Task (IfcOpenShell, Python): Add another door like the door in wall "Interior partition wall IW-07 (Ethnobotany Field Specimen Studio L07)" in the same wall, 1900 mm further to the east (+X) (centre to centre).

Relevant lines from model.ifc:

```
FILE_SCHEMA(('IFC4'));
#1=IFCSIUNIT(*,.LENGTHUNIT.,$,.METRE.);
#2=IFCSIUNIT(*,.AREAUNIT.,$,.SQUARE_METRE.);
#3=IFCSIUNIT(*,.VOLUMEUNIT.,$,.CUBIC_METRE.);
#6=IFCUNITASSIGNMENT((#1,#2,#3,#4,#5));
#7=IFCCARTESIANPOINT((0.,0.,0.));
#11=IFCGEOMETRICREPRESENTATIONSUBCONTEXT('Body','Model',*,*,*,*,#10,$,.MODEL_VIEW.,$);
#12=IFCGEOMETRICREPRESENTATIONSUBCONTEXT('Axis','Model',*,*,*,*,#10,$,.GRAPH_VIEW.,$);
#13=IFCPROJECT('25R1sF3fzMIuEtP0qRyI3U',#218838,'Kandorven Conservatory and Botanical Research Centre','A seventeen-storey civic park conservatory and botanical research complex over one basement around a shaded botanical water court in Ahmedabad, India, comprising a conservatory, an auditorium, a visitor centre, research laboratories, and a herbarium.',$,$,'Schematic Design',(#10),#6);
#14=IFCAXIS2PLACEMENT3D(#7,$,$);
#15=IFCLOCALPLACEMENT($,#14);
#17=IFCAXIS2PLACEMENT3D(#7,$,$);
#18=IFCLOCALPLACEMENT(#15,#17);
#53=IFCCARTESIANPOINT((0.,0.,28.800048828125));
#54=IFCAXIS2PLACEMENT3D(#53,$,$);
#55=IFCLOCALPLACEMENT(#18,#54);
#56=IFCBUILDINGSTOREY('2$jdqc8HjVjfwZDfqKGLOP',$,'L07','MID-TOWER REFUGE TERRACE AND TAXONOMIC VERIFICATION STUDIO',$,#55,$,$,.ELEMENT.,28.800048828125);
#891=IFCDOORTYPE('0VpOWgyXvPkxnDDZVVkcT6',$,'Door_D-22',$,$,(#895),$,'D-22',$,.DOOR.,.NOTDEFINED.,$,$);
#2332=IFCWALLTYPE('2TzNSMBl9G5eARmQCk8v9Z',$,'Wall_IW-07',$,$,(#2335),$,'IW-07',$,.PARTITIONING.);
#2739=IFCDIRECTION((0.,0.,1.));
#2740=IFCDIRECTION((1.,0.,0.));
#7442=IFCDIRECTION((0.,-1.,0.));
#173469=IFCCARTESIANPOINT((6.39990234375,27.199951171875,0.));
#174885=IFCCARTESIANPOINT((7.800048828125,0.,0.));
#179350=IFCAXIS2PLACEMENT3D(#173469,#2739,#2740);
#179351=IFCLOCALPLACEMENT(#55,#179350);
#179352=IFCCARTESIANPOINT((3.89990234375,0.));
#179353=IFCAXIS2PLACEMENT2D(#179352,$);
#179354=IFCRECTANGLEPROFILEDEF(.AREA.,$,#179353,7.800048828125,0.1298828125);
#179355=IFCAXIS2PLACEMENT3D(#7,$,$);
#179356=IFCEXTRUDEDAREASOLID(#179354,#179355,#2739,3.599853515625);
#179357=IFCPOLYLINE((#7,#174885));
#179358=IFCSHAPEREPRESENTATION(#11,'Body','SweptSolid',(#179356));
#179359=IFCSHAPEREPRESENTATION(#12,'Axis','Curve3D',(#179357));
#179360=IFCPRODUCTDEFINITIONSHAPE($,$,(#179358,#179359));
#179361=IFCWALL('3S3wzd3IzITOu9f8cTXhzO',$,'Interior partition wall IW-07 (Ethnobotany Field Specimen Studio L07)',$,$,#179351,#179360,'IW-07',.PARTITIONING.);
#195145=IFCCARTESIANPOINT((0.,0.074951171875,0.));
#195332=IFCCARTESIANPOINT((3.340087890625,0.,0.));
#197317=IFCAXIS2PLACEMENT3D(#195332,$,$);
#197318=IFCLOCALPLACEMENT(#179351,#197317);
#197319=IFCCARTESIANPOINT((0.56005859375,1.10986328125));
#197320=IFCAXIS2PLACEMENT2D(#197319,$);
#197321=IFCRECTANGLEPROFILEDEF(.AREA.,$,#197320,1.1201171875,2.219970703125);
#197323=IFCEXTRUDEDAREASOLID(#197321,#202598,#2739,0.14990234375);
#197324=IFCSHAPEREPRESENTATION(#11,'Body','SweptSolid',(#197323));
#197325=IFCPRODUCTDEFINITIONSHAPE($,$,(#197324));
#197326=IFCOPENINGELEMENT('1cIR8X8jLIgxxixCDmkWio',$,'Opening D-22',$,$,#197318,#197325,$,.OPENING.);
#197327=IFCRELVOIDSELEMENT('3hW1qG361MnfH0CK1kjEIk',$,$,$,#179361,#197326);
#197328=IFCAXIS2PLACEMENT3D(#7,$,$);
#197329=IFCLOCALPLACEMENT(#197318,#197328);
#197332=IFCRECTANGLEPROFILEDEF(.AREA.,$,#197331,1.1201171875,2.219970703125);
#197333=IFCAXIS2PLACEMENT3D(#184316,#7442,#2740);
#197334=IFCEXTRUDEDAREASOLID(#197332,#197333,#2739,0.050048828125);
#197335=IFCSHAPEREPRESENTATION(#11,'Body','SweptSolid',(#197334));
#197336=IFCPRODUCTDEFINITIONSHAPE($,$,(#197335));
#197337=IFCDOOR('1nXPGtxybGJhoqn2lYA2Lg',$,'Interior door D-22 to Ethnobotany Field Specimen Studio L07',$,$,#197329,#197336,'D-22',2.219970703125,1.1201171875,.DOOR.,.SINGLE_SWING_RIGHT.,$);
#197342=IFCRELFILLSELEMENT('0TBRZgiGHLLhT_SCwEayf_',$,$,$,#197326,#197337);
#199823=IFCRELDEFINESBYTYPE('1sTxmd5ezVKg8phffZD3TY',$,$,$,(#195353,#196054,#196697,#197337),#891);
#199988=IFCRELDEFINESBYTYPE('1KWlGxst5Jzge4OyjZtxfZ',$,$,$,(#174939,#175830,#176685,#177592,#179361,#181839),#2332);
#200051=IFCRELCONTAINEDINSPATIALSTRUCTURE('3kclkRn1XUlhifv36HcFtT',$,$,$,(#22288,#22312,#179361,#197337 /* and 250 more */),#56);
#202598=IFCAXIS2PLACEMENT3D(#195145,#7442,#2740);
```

```python
import ifcopenshell
import ifcopenshell.api.feature
import ifcopenshell.api.geometry
import ifcopenshell.api.root
import ifcopenshell.geom
import ifcopenshell.util.element
import ifcopenshell.util.placement
import ifcopenshell.util.shape

model = ifcopenshell.open("model.ifc")
settings = ifcopenshell.geom.settings()


def volume(element):
    """Net volume in cubic metres, openings subtracted."""
    shape = ifcopenshell.geom.create_shape(settings, element)
    return ifcopenshell.util.shape.get_volume(shape.geometry)


door = model.by_id(197337)
opening = door.FillsVoids[0].RelatingOpeningElement
wall = opening.VoidsElements[0].RelatingBuildingElement
before = volume(wall)
shift = ifcopenshell.util.placement.get_local_placement(wall.ObjectPlacement)[:3, 0] * 1.9

# copy_class copies the void relationship, type, container and properties, but no geometry.
new_opening = ifcopenshell.api.root.copy_class(model, product=opening)
new_opening.Representation = ifcopenshell.util.element.copy_deep(
    model, opening.Representation, exclude=["IfcGeometricRepresentationContext", "IfcRepresentationMap"]
)
new_door = ifcopenshell.api.root.copy_class(model, product=door)
new_door.Representation = ifcopenshell.util.element.copy_deep(
    model, door.Representation, exclude=["IfcGeometricRepresentationContext", "IfcRepresentationMap"]
)
new_door.Tag = None
ifcopenshell.api.feature.add_filling(model, opening=new_opening, element=new_door)

for old, new in ((opening, new_opening), (door, new_door)):
    matrix = ifcopenshell.util.placement.get_local_placement(old.ObjectPlacement)
    matrix[:3, 3] += shift
    ifcopenshell.api.geometry.edit_object_placement(model, product=new, matrix=matrix, is_si=False)

after = volume(wall)

print(f"wall volume {before:.3f} -> {after:.3f} m3")

model.write("model_v2.ifc")
```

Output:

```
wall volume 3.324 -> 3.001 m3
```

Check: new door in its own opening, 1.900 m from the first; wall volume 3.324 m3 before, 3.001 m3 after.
